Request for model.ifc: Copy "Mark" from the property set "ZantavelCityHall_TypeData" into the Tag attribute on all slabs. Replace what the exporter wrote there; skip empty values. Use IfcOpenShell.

First a look at what the model holds.

```python
import ifcopenshell
import ifcopenshell.util.element

model = ifcopenshell.open("model.ifc")
print(model.schema)
slabs = model.by_type("IfcSlab")
print(len(slabs), "slabs")
for e in slabs[:8]:
    source = ifcopenshell.util.element.get_pset(e, "ZantavelCityHall_TypeData", "Mark")
    target = e.Tag
    print(e.id(), repr(source), repr(target), sep=" | ")
```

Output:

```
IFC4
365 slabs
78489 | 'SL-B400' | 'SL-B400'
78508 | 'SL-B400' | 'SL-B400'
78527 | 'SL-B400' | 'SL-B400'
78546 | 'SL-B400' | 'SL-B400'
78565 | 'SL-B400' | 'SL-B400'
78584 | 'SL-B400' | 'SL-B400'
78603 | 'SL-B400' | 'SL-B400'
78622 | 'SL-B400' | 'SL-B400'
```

```python
import ifcopenshell
import ifcopenshell.util.element

model = ifcopenshell.open("model.ifc")

count = 0
for e in model.by_type("IfcSlab"):
    value = ifcopenshell.util.element.get_pset(e, "ZantavelCityHall_TypeData", "Mark")
    current = e.Tag
    if not value or not value.strip() or current == value:
        continue
    e.Tag = value
    count += 1

print(count, "slabs updated")

model.write("model_v2.ifc")
```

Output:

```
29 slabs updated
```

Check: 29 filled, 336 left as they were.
